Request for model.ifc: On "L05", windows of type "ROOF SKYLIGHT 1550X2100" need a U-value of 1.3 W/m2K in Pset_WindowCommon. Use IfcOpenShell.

First a look at what the model holds.

```python
import ifcopenshell
import ifcopenshell.util.element

model = ifcopenshell.open("model.ifc")
print(model.schema)
storey = next(s for s in model.by_type("IfcBuildingStorey") if s.Name == "L05")
windows = [e for e in ifcopenshell.util.element.get_decomposition(storey) if e.is_a("IfcWindow")]
seen = {}
for e in windows:
    element_type = ifcopenshell.util.element.get_type(e)
    key = (element_type.Name if element_type != e and element_type else None, ifcopenshell.util.element.get_pset(e, "Pset_WindowCommon", "ThermalTransmittance"))
    seen[key] = seen.get(key, 0) + 1
for (name, value), count in sorted(seen.items(), key=str):
    print(count, "x", name, "|", value)
```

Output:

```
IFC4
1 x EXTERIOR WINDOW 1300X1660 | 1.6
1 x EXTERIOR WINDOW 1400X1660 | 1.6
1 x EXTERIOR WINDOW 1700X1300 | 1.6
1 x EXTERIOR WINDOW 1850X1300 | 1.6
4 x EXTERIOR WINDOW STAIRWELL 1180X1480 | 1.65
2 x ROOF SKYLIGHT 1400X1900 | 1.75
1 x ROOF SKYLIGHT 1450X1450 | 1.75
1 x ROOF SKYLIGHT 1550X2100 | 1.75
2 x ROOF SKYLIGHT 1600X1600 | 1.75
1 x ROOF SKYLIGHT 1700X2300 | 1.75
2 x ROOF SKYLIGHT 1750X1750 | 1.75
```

```python
import ifcopenshell
import ifcopenshell.api.pset
import ifcopenshell.util.element

model = ifcopenshell.open("model.ifc")

storey = next(s for s in model.by_type("IfcBuildingStorey") if s.Name == "L05")
windows = [e for e in ifcopenshell.util.element.get_decomposition(storey) if e.is_a("IfcWindow")]

count = 0
for e in windows:
    element_type = ifcopenshell.util.element.get_type(e)
    if element_type in (None, e) or element_type.Name != "ROOF SKYLIGHT 1550X2100":
        continue
    # add_pset returns the element's existing set when there is one.
    pset = ifcopenshell.api.pset.add_pset(model, product=e, name="Pset_WindowCommon")
    ifcopenshell.api.pset.edit_pset(model, pset=pset, properties={"ThermalTransmittance": 1.3})
    count += 1

print(count, "windows updated")

model.write("model-out.ifc")
```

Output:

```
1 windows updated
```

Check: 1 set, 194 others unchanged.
